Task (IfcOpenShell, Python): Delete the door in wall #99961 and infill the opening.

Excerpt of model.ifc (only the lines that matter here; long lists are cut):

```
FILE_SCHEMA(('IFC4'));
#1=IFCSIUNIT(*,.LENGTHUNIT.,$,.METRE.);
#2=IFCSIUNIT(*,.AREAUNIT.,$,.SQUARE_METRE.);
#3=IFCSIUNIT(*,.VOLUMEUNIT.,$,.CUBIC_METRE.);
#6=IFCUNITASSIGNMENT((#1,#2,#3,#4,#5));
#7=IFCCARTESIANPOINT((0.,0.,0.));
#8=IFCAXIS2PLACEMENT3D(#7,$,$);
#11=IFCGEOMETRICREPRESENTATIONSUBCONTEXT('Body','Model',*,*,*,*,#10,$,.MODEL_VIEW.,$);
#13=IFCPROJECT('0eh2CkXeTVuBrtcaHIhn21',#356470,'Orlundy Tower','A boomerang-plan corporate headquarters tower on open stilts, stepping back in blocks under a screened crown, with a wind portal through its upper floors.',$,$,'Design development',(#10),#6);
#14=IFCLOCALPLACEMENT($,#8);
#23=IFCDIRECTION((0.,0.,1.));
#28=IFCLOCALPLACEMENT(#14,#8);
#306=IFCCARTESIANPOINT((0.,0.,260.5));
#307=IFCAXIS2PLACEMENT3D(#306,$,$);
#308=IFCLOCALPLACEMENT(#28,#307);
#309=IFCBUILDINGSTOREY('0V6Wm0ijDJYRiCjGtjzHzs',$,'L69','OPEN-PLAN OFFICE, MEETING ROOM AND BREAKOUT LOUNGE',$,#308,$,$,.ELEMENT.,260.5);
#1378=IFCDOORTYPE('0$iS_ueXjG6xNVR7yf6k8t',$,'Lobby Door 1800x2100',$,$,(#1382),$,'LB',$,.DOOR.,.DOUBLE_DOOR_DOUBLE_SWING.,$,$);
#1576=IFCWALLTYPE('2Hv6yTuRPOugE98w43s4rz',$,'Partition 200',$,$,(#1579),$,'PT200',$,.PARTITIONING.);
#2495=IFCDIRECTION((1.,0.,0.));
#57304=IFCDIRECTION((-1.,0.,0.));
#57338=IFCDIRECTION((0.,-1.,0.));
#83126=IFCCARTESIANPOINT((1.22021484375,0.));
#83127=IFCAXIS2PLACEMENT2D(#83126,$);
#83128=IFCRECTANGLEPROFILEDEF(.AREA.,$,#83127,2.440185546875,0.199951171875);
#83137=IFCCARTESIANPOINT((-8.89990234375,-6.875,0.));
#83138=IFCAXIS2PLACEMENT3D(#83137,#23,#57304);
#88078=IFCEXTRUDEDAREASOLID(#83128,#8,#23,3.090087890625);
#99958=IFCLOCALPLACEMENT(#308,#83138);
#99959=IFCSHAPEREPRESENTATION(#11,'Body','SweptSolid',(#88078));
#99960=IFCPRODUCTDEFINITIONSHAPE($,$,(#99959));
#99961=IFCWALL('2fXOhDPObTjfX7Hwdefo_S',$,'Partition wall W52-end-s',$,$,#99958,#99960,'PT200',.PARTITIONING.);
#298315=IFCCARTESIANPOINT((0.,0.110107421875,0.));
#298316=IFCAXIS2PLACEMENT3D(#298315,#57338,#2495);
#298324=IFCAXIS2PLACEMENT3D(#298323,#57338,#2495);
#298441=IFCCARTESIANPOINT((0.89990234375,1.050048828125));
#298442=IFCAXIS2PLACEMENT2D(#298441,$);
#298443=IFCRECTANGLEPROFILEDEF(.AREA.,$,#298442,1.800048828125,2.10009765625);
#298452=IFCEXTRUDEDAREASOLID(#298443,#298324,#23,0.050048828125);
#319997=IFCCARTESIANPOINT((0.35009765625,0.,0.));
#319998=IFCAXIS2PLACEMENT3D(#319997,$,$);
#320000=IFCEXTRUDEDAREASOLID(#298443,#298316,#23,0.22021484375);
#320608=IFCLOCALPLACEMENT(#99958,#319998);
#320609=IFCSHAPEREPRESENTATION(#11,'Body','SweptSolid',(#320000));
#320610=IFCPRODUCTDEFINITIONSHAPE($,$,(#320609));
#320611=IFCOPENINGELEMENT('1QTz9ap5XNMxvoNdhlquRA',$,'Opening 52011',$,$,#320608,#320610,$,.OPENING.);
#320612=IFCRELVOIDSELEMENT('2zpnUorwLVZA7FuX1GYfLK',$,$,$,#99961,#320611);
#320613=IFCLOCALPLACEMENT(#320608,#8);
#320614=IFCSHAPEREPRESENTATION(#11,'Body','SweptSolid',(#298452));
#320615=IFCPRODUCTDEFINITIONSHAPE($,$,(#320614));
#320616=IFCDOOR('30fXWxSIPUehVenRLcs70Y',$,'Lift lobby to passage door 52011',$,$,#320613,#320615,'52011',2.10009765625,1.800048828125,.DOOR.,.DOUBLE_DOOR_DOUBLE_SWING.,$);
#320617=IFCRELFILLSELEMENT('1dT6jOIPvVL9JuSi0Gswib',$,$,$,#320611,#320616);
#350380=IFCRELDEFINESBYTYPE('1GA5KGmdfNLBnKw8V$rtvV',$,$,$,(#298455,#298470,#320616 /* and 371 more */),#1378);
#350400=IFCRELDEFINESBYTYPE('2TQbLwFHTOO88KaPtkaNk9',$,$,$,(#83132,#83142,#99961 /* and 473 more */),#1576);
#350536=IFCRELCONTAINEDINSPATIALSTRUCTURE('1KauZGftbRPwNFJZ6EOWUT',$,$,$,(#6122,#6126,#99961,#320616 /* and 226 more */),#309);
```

```python
import ifcopenshell
import ifcopenshell.api.feature
import ifcopenshell.api.root
import ifcopenshell.geom
import ifcopenshell.util.shape

model = ifcopenshell.open("model.ifc")
settings = ifcopenshell.geom.settings()


def volume(element):
    """Net volume in cubic metres, openings subtracted."""
    shape = ifcopenshell.geom.create_shape(settings, element)
    return ifcopenshell.util.shape.get_volume(shape.geometry)


door = model.by_id(320616)
opening = door.FillsVoids[0].RelatingOpeningElement
wall = opening.VoidsElements[0].RelatingBuildingElement
before = volume(wall)

ifcopenshell.api.root.remove_product(model, product=door)
ifcopenshell.api.feature.remove_feature(model, feature=opening)

after = volume(wall)

print(f"wall volume {before:.3f} -> {after:.3f} m3")

model.write("model-out.ifc")
```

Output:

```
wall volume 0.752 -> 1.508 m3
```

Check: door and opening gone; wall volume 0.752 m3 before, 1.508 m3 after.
